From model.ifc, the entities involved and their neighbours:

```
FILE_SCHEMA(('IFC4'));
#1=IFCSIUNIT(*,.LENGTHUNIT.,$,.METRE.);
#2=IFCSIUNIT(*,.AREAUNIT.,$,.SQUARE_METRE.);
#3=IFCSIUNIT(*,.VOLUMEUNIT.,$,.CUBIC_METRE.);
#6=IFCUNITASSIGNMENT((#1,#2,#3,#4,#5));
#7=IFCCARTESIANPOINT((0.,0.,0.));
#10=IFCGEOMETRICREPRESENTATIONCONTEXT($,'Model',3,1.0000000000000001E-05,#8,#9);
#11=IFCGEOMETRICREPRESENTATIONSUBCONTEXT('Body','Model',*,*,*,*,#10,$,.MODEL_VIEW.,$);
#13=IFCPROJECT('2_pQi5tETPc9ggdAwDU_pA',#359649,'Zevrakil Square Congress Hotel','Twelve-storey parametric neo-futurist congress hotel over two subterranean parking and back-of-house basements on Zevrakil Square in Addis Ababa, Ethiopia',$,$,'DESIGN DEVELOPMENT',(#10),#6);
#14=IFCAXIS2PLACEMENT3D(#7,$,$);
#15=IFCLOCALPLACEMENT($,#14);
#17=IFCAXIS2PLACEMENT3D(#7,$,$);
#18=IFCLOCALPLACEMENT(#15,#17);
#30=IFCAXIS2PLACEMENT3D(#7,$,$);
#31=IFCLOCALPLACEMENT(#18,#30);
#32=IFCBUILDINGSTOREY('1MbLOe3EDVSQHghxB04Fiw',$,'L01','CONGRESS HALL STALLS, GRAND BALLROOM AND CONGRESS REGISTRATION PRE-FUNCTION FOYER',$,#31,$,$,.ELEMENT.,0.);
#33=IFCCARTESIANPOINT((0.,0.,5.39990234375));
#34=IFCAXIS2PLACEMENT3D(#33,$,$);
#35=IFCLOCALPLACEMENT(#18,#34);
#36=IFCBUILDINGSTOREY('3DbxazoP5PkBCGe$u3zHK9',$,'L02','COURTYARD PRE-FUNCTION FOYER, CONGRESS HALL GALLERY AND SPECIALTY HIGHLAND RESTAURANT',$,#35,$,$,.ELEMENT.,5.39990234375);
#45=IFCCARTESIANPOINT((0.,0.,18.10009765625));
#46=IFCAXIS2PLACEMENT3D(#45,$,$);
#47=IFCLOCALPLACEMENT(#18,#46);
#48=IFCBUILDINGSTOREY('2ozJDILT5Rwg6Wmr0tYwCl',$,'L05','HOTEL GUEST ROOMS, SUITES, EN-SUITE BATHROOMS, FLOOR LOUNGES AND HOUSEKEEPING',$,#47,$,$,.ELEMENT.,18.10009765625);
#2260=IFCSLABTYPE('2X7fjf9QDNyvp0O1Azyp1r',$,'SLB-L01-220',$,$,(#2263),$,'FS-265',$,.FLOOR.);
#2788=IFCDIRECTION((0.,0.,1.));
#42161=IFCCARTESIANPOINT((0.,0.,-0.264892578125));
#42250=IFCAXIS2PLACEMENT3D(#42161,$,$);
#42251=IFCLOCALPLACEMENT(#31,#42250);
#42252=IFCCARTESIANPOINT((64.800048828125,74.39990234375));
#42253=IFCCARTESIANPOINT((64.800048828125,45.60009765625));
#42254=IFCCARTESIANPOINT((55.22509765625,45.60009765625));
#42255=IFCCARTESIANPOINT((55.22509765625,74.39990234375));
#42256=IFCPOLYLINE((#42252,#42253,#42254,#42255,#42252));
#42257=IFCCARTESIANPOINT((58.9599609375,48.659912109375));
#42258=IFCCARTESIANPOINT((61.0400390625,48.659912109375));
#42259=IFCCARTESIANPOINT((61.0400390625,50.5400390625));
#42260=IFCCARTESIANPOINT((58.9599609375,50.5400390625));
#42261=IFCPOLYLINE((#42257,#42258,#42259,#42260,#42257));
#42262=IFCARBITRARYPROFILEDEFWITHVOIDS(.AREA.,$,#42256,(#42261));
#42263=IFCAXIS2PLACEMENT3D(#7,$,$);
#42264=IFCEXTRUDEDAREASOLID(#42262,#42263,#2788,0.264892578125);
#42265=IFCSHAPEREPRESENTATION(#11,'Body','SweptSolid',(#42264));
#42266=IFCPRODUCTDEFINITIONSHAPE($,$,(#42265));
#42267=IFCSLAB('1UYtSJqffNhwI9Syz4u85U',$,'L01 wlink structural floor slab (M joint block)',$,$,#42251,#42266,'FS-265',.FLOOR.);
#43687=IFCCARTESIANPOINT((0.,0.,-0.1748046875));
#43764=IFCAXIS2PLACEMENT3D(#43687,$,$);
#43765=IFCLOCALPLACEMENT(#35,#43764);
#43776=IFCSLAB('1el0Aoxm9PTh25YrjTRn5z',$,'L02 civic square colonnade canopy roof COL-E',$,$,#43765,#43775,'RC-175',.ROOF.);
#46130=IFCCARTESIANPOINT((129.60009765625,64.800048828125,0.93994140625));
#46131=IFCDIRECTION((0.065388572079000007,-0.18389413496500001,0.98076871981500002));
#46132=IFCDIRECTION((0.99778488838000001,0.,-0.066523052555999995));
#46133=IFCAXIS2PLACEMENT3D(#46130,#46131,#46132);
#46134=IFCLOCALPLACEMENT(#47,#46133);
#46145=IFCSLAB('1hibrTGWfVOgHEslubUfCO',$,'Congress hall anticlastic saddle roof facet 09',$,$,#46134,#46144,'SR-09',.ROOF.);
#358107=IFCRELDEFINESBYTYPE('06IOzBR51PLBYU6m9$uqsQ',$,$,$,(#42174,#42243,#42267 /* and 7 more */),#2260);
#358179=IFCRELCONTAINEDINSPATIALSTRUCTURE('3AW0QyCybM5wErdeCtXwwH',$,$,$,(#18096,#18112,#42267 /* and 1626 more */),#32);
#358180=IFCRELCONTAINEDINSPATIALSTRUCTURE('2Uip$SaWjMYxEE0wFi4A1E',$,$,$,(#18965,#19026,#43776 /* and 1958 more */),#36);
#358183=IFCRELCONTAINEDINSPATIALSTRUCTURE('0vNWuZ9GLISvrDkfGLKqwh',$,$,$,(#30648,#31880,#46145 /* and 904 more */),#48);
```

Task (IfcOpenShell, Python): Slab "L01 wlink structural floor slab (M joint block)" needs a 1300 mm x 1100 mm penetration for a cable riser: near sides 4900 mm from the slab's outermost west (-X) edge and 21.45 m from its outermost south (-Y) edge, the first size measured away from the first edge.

```python
import numpy as np
import ifcopenshell
import ifcopenshell.api.feature
import ifcopenshell.api.geometry
import ifcopenshell.api.root
import ifcopenshell.geom
import ifcopenshell.util.placement
import ifcopenshell.util.representation
import ifcopenshell.util.shape
import ifcopenshell.util.unit

model = ifcopenshell.open("model.ifc")
unit_scale = ifcopenshell.util.unit.calculate_unit_scale(model)
settings = ifcopenshell.geom.settings()


def volume(element):
    """Net volume in cubic metres, openings subtracted."""
    shape = ifcopenshell.geom.create_shape(settings, element)
    return ifcopenshell.util.shape.get_volume(shape.geometry)


slab = model.by_guid("1UYtSJqffNhwI9Syz4u85U")
before = volume(slab)

# Extent in the slab's own axes, in metres. The edges named are its -X and -Y sides.
slab_shape = ifcopenshell.geom.create_shape(settings, slab)
vertices = ifcopenshell.util.shape.get_vertices(slab_shape.geometry)
x_min, y_min, bottom = vertices.min(axis=0)
top = vertices[:, 2].max()

opening = ifcopenshell.api.root.create_entity(model, ifc_class="IfcOpeningElement", name="Cable riser opening", predefined_type="OPENING")
context = ifcopenshell.util.representation.get_context(model, "Model", "Body", "MODEL_VIEW")
width, depth = 1.3, 1.1
outline = [(0.0, 0.0), (width, 0.0), (width, depth), (0.0, depth), (0.0, 0.0)]
# Overshoot both faces by 50 mm so the cut is clean.
shape = ifcopenshell.api.geometry.add_slab_representation(
    model, context=context, depth=top - bottom + 0.1, polyline=outline
)
ifcopenshell.api.geometry.assign_representation(model, product=opening, representation=shape)

matrix = ifcopenshell.util.placement.get_local_placement(slab.ObjectPlacement)
matrix[:, 3] = matrix @ np.append(np.array([x_min + 4.9, y_min + 21.45, bottom - 0.05]) / unit_scale, 1.0)
ifcopenshell.api.geometry.edit_object_placement(model, product=opening, matrix=matrix, is_si=False)
ifcopenshell.api.feature.add_feature(model, feature=opening, element=slab)

after = volume(slab)

print(f"slab volume {before:.3f} -> {after:.3f} m3")

model.write("model_updated.ifc")
```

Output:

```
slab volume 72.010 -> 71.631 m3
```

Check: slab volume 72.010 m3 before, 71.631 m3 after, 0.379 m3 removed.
